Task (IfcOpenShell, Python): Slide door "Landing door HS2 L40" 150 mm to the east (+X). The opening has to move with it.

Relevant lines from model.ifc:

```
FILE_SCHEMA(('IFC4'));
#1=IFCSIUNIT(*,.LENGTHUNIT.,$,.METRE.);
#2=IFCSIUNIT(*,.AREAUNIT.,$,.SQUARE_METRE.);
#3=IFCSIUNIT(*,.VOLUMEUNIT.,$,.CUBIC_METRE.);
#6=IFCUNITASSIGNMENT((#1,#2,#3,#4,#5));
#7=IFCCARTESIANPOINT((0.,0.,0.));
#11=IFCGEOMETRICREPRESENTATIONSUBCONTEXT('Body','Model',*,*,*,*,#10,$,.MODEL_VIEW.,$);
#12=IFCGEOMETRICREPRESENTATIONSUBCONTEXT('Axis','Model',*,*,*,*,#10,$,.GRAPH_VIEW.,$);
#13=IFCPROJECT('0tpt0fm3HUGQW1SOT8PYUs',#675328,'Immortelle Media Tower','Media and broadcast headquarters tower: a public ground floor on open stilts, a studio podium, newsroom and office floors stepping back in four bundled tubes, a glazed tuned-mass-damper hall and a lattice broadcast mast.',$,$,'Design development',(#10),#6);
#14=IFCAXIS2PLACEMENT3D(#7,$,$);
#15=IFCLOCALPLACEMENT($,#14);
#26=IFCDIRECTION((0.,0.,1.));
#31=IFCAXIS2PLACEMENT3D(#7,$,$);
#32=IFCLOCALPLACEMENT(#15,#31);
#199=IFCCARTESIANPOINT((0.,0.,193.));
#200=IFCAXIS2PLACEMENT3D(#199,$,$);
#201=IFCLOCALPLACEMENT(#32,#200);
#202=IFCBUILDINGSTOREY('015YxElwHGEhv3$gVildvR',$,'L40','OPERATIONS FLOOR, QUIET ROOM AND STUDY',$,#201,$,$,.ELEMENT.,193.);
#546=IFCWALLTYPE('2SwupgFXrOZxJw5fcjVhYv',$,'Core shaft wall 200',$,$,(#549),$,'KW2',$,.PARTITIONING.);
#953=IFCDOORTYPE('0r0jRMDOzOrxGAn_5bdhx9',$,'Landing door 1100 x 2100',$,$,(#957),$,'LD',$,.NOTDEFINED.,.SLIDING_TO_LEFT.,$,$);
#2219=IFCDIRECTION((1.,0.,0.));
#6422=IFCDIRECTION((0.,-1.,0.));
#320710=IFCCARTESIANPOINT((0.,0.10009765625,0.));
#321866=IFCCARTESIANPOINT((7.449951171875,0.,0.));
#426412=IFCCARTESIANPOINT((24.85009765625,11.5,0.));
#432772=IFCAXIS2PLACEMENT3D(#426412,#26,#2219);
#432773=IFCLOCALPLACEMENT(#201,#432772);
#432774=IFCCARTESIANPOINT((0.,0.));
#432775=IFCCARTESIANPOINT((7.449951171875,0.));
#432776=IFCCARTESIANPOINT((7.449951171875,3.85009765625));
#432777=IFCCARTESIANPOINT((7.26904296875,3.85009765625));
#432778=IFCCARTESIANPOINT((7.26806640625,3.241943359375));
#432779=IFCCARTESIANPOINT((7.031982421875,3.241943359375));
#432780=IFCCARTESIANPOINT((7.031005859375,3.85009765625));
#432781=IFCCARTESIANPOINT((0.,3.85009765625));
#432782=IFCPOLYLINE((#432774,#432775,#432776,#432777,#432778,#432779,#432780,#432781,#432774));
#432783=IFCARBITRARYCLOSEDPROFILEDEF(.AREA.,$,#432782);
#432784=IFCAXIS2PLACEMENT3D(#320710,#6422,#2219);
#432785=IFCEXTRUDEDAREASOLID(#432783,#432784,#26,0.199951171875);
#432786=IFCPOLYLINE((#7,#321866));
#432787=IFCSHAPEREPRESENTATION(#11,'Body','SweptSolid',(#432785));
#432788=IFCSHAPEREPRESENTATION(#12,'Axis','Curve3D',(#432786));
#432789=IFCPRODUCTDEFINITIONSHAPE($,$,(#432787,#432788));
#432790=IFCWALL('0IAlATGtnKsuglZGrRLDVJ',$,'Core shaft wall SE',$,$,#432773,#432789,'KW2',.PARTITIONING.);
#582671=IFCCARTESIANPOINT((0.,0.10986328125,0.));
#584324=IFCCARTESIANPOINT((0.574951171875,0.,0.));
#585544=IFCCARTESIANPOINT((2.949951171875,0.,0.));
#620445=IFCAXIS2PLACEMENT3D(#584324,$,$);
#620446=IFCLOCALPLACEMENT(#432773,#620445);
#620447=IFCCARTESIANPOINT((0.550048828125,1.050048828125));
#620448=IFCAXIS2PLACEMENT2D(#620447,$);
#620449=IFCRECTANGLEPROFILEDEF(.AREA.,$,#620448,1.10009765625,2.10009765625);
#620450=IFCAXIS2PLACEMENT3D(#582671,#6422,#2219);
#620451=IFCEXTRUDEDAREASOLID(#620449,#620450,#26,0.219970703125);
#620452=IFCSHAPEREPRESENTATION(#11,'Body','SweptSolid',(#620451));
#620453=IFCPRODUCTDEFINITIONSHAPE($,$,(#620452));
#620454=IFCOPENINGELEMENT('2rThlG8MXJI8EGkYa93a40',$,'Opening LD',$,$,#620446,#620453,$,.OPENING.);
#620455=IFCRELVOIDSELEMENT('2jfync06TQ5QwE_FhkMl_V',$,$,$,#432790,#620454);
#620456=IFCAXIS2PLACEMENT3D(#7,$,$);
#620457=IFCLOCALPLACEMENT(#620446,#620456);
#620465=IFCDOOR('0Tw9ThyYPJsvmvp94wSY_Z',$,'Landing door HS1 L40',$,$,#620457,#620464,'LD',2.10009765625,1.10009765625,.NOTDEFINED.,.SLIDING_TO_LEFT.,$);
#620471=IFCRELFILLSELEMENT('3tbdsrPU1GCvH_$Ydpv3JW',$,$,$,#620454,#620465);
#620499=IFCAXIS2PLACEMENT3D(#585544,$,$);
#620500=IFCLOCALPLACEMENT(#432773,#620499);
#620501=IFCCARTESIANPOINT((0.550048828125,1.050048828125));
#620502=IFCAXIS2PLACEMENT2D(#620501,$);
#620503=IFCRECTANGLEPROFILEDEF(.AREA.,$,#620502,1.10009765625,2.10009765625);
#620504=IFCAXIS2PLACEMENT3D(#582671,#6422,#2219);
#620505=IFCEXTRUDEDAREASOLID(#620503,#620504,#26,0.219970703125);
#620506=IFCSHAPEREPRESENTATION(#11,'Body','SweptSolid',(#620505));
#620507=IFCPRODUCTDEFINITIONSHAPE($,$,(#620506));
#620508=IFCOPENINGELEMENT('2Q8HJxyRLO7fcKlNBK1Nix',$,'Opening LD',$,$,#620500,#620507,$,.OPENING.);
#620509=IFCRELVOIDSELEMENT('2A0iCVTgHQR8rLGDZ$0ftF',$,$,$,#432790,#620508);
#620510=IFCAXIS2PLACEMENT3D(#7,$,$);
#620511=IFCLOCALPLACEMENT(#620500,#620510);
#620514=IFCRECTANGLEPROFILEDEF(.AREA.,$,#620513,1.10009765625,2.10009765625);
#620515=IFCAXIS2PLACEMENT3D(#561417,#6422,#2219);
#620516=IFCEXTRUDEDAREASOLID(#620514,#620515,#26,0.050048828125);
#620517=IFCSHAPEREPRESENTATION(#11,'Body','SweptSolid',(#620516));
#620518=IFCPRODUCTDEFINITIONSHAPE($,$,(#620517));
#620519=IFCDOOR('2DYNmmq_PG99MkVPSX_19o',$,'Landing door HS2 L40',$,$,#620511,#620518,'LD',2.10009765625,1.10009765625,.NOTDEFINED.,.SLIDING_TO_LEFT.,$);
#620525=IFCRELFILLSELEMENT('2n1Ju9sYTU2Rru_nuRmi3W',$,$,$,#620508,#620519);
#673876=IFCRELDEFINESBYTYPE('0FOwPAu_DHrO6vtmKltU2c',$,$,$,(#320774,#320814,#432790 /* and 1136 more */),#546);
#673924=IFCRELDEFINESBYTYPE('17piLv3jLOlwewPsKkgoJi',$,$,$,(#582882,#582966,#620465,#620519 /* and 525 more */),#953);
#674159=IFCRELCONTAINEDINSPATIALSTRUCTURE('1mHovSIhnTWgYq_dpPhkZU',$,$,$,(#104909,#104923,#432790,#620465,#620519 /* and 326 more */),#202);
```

```python
import ifcopenshell
import ifcopenshell.api.geometry
import ifcopenshell.util.placement
import ifcopenshell.util.unit

model = ifcopenshell.open("model.ifc")
unit_scale = ifcopenshell.util.unit.calculate_unit_scale(model)

door = model.by_guid("2DYNmmq_PG99MkVPSX_19o")
opening = door.FillsVoids[0].RelatingOpeningElement
wall = opening.VoidsElements[0].RelatingBuildingElement

wall_matrix = ifcopenshell.util.placement.get_local_placement(wall.ObjectPlacement)
shift = wall_matrix[:3, 0] * 0.15 / unit_scale
before = ifcopenshell.util.placement.get_local_placement(door.ObjectPlacement)[:3, 3].copy()

# The door is placed relative to its opening, so it follows when the opening moves.
matrix = ifcopenshell.util.placement.get_local_placement(opening.ObjectPlacement)
matrix[:3, 3] += shift
ifcopenshell.api.geometry.edit_object_placement(
    model, product=opening, matrix=matrix, is_si=False, should_transform_children=True
)

after = ifcopenshell.util.placement.get_local_placement(door.ObjectPlacement)[:3, 3]
print("door moved by", (after - before).round(3) + 0.0)

model.write("model_rev.ifc")
```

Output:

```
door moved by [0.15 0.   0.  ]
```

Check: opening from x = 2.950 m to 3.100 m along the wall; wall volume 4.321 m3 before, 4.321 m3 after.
